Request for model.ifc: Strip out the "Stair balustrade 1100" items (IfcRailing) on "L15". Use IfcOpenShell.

First a look at what the model holds.

```python
import ifcopenshell
import ifcopenshell.util.element

model = ifcopenshell.open("model.ifc")
print(model.schema)
storey = next(s for s in model.by_type("IfcBuildingStorey") if s.Name == "L15")
railings = [e for e in ifcopenshell.util.element.get_decomposition(storey) if e.is_a("IfcRailing")]
seen = {}
for e in railings:
    element_type = ifcopenshell.util.element.get_type(e)
    name = element_type.Name if element_type not in (None, e) else None
    seen[name] = seen.get(name, 0) + 1
for name, count in sorted(seen.items(), key=str):
    print(count, "x", name)
```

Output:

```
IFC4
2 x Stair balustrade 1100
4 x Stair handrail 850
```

```python
import ifcopenshell
import ifcopenshell.api.root
import ifcopenshell.util.element

model = ifcopenshell.open("model.ifc")

storey = next(s for s in model.by_type("IfcBuildingStorey") if s.Name == "L15")
railings = [e for e in ifcopenshell.util.element.get_decomposition(storey) if e.is_a("IfcRailing")]
targets = [e for e in railings if (t := ifcopenshell.util.element.get_type(e)) not in (None, e) and t.Name == "Stair balustrade 1100"]

for e in targets:
    ifcopenshell.api.root.remove_product(model, product=e)
print(len(targets), "removed")

model.write("model-out.ifc")
```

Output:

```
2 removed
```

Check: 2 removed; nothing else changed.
